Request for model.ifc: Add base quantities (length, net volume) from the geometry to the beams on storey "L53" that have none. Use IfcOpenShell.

First a look at what the model holds.

```python
import ifcopenshell
import ifcopenshell.util.element
import ifcopenshell.util.unit

model = ifcopenshell.open("model.ifc")
print(model.schema)
for unit_type in ("LENGTHUNIT", "AREAUNIT", "VOLUMEUNIT"):
    print(unit_type, ifcopenshell.util.unit.calculate_unit_scale(model, unit_type))
storey = next(s for s in model.by_type("IfcBuildingStorey") if s.Name == "L53")
beams = [e for e in ifcopenshell.util.element.get_decomposition(storey) if e.is_a("IfcBeam")]
for e in sorted(beams, key=lambda e: e.id()):
    print(e.id(), e.is_a(), e.Name, list(ifcopenshell.util.element.get_psets(e, qtos_only=True)), sep=" | ")
```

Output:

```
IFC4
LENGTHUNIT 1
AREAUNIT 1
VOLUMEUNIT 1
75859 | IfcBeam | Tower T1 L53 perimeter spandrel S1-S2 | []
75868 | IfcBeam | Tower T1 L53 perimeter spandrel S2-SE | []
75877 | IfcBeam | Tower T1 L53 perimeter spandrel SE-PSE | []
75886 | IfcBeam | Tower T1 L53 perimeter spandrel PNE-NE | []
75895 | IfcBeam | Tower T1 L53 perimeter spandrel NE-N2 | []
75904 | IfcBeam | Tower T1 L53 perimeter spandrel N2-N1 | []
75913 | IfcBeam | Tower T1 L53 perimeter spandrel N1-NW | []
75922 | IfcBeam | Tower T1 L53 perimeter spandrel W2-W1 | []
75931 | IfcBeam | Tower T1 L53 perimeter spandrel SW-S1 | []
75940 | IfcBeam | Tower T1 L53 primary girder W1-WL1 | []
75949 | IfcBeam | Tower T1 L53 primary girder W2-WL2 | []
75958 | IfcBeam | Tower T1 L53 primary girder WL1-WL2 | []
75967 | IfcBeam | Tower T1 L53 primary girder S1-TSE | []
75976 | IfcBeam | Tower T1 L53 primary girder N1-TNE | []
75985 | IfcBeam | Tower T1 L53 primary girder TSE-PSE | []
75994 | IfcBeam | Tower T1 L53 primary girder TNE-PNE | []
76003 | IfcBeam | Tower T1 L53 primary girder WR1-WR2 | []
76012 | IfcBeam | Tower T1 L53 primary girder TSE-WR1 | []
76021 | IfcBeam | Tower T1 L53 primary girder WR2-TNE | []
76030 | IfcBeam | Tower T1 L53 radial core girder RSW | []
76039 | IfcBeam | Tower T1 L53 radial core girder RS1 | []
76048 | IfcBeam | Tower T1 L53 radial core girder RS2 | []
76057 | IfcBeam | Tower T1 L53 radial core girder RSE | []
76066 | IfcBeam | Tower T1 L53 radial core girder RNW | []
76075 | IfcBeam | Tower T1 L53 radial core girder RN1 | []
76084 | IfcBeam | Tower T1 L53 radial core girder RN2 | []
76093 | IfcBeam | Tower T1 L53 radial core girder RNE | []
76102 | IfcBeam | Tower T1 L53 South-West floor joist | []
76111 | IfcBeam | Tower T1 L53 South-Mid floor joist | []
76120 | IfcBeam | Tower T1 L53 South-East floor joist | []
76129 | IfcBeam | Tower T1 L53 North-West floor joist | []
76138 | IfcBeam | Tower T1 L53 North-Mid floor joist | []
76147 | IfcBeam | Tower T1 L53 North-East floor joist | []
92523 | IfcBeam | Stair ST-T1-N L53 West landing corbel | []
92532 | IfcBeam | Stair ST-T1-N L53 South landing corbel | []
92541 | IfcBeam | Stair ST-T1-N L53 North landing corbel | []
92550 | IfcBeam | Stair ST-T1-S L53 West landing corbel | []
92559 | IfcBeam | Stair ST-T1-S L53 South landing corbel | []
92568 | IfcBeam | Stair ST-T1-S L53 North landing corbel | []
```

```python
import ifcopenshell
import ifcopenshell.api.pset
import ifcopenshell.geom
import ifcopenshell.util.element
import ifcopenshell.util.shape
import ifcopenshell.util.unit

model = ifcopenshell.open("model.ifc")
unit_scale = ifcopenshell.util.unit.calculate_unit_scale(model)
volume_scale = ifcopenshell.util.unit.calculate_unit_scale(model, "VOLUMEUNIT")
settings = ifcopenshell.geom.settings()

storey = next(s for s in model.by_type("IfcBuildingStorey") if s.Name == "L53")
beams = [e for e in ifcopenshell.util.element.get_decomposition(storey) if e.is_a("IfcBeam")]

for e in sorted(beams, key=lambda e: e.id()):
    if ifcopenshell.util.element.get_psets(e, qtos_only=True, should_inherit=False):
        continue
    # Geometry comes back in metres, in the element's own axes.
    shape = ifcopenshell.geom.create_shape(settings, e)
    values = {
        "Length": ifcopenshell.util.shape.get_max_xyz(shape.geometry) / unit_scale,
        "NetVolume": ifcopenshell.util.shape.get_volume(shape.geometry) / volume_scale,
    }
    qto = ifcopenshell.api.pset.add_qto(model, product=e, name="Qto_BeamBaseQuantities")
    ifcopenshell.api.pset.edit_qto(model, qto=qto, properties=values)
    print(e.id(), {k: round(v, 3) for k, v in values.items()})

model.write("model_rev.ifc")
```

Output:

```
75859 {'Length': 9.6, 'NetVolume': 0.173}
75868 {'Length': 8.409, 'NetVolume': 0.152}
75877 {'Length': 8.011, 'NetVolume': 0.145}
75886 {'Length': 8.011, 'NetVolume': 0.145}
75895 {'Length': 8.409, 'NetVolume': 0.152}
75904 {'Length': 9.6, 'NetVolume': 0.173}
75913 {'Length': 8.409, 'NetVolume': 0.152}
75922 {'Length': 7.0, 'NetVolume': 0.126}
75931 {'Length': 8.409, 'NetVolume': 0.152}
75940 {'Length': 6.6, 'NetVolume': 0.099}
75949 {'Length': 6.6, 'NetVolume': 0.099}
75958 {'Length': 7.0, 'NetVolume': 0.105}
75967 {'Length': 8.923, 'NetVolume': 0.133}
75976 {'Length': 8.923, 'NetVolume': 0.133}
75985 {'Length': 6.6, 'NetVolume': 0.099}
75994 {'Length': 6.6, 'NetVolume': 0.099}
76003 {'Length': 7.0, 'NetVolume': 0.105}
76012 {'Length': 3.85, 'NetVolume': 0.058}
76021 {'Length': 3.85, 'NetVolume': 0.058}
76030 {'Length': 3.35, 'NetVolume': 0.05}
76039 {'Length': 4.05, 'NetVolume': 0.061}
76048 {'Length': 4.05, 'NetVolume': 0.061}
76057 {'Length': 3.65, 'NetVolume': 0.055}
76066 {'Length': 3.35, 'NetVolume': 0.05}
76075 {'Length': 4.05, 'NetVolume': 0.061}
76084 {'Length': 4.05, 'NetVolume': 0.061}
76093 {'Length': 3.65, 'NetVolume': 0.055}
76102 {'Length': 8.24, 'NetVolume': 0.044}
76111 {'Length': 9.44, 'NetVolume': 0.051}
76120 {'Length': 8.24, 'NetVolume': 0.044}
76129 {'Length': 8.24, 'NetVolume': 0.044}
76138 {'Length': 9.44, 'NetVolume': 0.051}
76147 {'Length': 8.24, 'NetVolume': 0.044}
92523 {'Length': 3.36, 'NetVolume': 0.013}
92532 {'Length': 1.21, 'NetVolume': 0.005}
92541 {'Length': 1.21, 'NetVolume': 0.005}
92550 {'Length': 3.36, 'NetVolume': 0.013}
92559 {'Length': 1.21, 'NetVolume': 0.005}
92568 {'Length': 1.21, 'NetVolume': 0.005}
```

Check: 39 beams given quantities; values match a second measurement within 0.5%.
